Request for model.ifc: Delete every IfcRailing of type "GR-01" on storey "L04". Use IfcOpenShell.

First a look at what the model holds.

```python
import ifcopenshell
import ifcopenshell.util.element

model = ifcopenshell.open("model.ifc")
print(model.schema)
storey = next(s for s in model.by_type("IfcBuildingStorey") if s.Name == "L04")
railings = [e for e in ifcopenshell.util.element.get_decomposition(storey) if e.is_a("IfcRailing")]
seen = {}
for e in railings:
    element_type = ifcopenshell.util.element.get_type(e)
    name = element_type.Name if element_type not in (None, e) else None
    seen[name] = seen.get(name, 0) + 1
for name, count in sorted(seen.items(), key=str):
    print(count, "x", name)
```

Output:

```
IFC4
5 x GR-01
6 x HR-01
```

```python
import ifcopenshell
import ifcopenshell.api.root
import ifcopenshell.util.element

model = ifcopenshell.open("model.ifc")

storey = next(s for s in model.by_type("IfcBuildingStorey") if s.Name == "L04")
railings = [e for e in ifcopenshell.util.element.get_decomposition(storey) if e.is_a("IfcRailing")]
targets = [e for e in railings if (t := ifcopenshell.util.element.get_type(e)) not in (None, e) and t.Name == "GR-01"]

for e in targets:
    ifcopenshell.api.root.remove_product(model, product=e)
print(len(targets), "removed")

model.write("model_updated.ifc")
```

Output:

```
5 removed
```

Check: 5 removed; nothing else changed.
